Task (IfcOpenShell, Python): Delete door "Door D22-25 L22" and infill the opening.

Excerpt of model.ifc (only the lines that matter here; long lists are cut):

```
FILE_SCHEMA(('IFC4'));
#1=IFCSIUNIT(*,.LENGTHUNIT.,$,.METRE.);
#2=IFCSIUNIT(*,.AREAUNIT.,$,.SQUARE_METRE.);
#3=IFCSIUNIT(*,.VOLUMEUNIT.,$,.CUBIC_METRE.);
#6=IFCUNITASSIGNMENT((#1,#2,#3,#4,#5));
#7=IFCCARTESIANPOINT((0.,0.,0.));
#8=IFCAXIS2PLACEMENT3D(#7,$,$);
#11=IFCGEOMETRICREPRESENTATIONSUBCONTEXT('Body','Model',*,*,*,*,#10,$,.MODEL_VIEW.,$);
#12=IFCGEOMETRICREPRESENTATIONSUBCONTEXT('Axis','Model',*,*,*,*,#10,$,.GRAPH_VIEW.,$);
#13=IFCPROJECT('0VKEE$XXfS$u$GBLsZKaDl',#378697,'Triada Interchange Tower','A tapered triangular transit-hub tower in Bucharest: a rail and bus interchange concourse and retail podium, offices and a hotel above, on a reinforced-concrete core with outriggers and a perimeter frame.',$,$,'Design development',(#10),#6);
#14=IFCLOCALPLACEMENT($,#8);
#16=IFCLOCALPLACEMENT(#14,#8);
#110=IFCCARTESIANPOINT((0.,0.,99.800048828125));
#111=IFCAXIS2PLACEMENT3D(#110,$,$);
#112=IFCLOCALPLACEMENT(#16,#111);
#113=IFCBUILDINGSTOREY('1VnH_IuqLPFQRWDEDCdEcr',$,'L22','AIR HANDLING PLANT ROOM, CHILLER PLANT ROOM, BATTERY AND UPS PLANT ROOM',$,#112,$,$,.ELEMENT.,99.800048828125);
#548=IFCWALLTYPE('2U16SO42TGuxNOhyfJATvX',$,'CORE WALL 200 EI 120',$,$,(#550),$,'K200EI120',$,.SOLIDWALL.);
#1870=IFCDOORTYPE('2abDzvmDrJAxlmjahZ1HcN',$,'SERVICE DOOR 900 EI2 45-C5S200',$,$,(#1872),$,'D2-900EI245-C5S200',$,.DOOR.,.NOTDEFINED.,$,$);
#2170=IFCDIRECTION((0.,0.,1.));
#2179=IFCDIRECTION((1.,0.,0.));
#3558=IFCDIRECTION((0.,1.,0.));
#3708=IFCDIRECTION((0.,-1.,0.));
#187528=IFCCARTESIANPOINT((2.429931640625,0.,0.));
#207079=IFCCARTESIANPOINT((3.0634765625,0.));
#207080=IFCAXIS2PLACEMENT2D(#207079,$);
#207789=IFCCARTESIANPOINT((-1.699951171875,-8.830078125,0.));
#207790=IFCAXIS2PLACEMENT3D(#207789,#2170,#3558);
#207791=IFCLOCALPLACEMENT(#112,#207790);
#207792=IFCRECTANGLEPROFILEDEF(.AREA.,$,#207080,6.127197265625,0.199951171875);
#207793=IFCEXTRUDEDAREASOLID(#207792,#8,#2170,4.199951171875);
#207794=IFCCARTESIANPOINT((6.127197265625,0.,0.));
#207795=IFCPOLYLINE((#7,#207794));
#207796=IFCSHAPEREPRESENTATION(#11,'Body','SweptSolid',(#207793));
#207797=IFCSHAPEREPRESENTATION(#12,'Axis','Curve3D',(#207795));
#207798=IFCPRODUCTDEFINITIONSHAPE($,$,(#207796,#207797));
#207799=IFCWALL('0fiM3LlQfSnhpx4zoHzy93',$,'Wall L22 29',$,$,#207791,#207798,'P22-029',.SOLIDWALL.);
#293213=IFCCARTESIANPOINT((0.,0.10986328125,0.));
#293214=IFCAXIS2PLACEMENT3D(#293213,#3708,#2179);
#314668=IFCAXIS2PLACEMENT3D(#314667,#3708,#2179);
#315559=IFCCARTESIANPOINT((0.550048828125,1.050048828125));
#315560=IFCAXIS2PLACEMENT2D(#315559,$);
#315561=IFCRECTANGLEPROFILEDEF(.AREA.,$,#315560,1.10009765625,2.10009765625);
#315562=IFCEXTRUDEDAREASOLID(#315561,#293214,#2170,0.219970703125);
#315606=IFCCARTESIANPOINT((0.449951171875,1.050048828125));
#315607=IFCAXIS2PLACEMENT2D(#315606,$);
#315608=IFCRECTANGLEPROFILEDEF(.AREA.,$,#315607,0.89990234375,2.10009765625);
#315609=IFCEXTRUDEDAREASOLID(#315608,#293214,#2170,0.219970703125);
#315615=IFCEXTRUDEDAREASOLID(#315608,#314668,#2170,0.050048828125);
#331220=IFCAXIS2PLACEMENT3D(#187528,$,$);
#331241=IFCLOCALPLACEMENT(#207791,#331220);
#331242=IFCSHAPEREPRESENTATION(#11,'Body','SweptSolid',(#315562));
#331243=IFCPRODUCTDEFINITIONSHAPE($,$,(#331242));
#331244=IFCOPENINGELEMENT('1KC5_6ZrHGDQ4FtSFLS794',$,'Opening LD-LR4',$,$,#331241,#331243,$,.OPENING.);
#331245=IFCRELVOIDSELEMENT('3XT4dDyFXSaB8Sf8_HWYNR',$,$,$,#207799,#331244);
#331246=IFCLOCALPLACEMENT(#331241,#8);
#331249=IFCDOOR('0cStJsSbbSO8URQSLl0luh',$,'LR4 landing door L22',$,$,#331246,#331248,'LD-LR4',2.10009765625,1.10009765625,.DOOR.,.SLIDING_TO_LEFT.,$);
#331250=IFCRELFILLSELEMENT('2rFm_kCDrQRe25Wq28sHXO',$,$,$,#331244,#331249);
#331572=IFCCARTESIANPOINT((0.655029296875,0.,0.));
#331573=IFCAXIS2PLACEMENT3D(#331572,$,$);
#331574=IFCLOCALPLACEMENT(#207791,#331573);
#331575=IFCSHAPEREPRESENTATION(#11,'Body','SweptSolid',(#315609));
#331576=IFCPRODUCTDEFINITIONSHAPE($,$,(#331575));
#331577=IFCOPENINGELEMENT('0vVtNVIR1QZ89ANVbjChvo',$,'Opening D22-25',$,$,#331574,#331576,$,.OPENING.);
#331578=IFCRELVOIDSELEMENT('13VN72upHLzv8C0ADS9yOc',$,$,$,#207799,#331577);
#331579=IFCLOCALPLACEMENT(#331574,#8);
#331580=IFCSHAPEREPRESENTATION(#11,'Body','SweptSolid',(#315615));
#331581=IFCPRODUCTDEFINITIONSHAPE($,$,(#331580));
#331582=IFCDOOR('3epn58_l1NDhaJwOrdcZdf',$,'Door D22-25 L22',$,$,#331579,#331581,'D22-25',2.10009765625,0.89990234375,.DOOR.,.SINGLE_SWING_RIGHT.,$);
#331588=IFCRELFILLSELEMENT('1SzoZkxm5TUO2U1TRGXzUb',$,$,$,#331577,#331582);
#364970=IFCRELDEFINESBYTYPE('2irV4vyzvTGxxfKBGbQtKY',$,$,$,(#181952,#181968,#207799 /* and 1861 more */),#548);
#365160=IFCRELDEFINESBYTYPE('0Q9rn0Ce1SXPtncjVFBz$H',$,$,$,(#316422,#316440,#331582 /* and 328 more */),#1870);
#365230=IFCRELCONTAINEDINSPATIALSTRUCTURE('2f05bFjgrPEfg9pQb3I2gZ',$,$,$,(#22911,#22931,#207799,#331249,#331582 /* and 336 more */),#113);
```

```python
import ifcopenshell
import ifcopenshell.api.feature
import ifcopenshell.api.root
import ifcopenshell.geom
import ifcopenshell.util.shape

model = ifcopenshell.open("model.ifc")
settings = ifcopenshell.geom.settings()


def volume(element):
    """Net volume in cubic metres, openings subtracted."""
    shape = ifcopenshell.geom.create_shape(settings, element)
    return ifcopenshell.util.shape.get_volume(shape.geometry)


door = model.by_guid("3epn58_l1NDhaJwOrdcZdf")
opening = door.FillsVoids[0].RelatingOpeningElement
wall = opening.VoidsElements[0].RelatingBuildingElement
before = volume(wall)

ifcopenshell.api.root.remove_product(model, product=door)
ifcopenshell.api.feature.remove_feature(model, feature=opening)

after = volume(wall)

print(f"wall volume {before:.3f} -> {after:.3f} m3")

model.write("model-out.ifc")
```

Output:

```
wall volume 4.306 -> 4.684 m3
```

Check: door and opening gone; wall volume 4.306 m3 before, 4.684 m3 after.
